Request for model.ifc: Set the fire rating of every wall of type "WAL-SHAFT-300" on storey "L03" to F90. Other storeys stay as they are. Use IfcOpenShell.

First a look at what the model holds.

```python
import ifcopenshell
import ifcopenshell.util.element

model = ifcopenshell.open("model.ifc")
print(model.schema)
storey = next(s for s in model.by_type("IfcBuildingStorey") if s.Name == "L03")
walls = [e for e in ifcopenshell.util.element.get_decomposition(storey) if e.is_a("IfcWall")]
seen = {}
for e in walls:
    element_type = ifcopenshell.util.element.get_type(e)
    key = (element_type.Name if element_type != e and element_type else None, ifcopenshell.util.element.get_pset(e, "Pset_WallCommon", "FireRating"))
    seen[key] = seen.get(key, 0) + 1
for (name, value), count in sorted(seen.items(), key=str):
    print(count, "x", name, "|", value)
```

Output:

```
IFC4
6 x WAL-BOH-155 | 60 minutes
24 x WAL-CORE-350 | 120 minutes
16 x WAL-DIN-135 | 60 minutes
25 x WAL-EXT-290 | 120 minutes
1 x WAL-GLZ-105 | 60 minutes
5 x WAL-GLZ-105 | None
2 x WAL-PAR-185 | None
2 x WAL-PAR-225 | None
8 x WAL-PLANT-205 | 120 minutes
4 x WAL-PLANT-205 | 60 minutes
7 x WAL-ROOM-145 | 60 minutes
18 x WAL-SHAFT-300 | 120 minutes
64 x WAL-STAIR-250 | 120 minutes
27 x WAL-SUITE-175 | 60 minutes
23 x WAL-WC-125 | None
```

```python
import ifcopenshell
import ifcopenshell.api.pset
import ifcopenshell.util.element

model = ifcopenshell.open("model.ifc")

storey = next(s for s in model.by_type("IfcBuildingStorey") if s.Name == "L03")
walls = [e for e in ifcopenshell.util.element.get_decomposition(storey) if e.is_a("IfcWall")]

count = 0
for e in walls:
    element_type = ifcopenshell.util.element.get_type(e)
    if element_type in (None, e) or element_type.Name != "WAL-SHAFT-300":
        continue
    # add_pset returns the element's existing set when there is one.
    pset = ifcopenshell.api.pset.add_pset(model, product=e, name="Pset_WallCommon")
    ifcopenshell.api.pset.edit_pset(model, pset=pset, properties={"FireRating": "F90"})
    count += 1

print(count, "walls updated")

model.write("model_edited.ifc")
```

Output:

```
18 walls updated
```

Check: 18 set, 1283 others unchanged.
